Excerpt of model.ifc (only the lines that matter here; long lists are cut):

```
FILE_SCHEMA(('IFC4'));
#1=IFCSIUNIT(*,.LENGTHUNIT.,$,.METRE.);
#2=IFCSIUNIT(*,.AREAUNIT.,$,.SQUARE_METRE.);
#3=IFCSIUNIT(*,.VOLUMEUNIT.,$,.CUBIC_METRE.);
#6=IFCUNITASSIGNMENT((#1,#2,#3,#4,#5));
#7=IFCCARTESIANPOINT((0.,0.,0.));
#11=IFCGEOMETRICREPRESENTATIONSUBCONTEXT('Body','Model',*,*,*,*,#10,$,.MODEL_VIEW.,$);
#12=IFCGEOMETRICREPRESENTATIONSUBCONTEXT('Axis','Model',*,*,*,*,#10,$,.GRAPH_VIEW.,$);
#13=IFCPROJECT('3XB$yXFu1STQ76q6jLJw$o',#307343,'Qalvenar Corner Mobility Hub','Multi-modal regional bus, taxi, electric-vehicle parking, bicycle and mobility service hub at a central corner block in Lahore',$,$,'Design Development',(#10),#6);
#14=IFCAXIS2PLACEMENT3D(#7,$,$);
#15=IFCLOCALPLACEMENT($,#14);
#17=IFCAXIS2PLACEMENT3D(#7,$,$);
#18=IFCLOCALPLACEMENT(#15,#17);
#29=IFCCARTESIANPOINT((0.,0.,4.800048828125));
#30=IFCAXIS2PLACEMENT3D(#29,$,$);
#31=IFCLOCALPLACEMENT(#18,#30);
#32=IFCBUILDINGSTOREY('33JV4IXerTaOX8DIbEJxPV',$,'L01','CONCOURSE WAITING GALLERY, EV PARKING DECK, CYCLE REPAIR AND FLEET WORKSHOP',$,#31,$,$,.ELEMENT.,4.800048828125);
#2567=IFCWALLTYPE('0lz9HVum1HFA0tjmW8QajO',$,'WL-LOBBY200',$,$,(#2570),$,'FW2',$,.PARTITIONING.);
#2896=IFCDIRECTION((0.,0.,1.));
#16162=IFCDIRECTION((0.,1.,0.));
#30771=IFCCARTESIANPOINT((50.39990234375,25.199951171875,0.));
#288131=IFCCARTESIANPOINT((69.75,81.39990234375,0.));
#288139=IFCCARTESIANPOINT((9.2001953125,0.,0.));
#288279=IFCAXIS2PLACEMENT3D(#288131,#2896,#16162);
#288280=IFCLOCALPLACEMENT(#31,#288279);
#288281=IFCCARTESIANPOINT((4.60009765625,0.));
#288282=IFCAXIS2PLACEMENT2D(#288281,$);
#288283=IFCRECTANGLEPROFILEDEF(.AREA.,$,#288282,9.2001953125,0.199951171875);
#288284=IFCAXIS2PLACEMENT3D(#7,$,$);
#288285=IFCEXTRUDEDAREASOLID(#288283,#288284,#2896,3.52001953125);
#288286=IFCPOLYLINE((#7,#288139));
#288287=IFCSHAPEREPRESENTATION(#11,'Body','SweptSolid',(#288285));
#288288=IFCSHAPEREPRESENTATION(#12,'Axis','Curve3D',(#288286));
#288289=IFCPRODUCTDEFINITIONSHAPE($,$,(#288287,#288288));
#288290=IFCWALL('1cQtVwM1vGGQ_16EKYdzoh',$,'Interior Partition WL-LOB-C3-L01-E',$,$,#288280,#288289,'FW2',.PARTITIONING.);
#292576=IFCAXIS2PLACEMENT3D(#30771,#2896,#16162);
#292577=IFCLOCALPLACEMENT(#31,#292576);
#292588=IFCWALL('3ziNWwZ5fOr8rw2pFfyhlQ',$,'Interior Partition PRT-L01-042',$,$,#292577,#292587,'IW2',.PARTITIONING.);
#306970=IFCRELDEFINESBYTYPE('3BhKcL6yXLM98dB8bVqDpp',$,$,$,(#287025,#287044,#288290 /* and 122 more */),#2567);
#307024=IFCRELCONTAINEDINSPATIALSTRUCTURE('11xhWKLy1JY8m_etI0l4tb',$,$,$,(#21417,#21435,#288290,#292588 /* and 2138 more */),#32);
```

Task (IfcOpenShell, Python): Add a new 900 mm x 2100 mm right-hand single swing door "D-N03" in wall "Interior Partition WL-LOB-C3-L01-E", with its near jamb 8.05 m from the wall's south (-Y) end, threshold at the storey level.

```python
import numpy as np
import ifcopenshell
import ifcopenshell.api.feature
import ifcopenshell.api.geometry
import ifcopenshell.api.root
import ifcopenshell.api.spatial
import ifcopenshell.geom
import ifcopenshell.util.element
import ifcopenshell.util.placement
import ifcopenshell.util.representation
import ifcopenshell.util.shape
import ifcopenshell.util.unit

model = ifcopenshell.open("model.ifc")
unit_scale = ifcopenshell.util.unit.calculate_unit_scale(model)
settings = ifcopenshell.geom.settings()


def volume(element):
    """Net volume in cubic metres, openings subtracted."""
    shape = ifcopenshell.geom.create_shape(settings, element)
    return ifcopenshell.util.shape.get_volume(shape.geometry)


wall = model.by_guid("1cQtVwM1vGGQ_16EKYdzoh")
storey = ifcopenshell.util.element.get_container(wall, ifc_class="IfcBuildingStorey")
context = ifcopenshell.util.representation.get_context(model, "Model", "Body", "MODEL_VIEW")
before = volume(wall)

width, height, from_end, sill = 0.9, 2.1, 8.05, 0.0  # metres

# The wall runs along its own X axis, and the end named is its -X end.
wall_shape = ifcopenshell.geom.create_shape(settings, wall)
x, y, z = ifcopenshell.util.shape.get_vertices(wall_shape.geometry).T
start = x.min() + from_end
face, thickness = float(y.min()), float(y.max() - y.min())
wall_matrix = ifcopenshell.util.placement.get_local_placement(wall.ObjectPlacement)
level = ifcopenshell.util.placement.get_local_placement(storey.ObjectPlacement)[2, 3]


def in_wall(x, y):
    """Placement at x, y metres in the wall's axes, at sill height."""
    matrix = wall_matrix.copy()
    matrix[:, 3] = wall_matrix @ np.array([x / unit_scale, y / unit_scale, 0.0, 1.0])
    matrix[2, 3] = level + sill / unit_scale
    return matrix


# Opening: a box that overshoots both wall faces by 50 mm.
opening = ifcopenshell.api.root.create_entity(model, ifc_class="IfcOpeningElement", predefined_type="OPENING")
box = ifcopenshell.api.geometry.add_wall_representation(
    model, context=context, length=width, height=height, thickness=thickness + 0.1
)
ifcopenshell.api.geometry.assign_representation(model, product=opening, representation=box)
ifcopenshell.api.geometry.edit_object_placement(model, product=opening, matrix=in_wall(start, face - 0.05), is_si=False)
ifcopenshell.api.feature.add_feature(model, feature=opening, element=wall)

door = ifcopenshell.api.root.create_entity(model, ifc_class="IfcDoor", name="D-N03", predefined_type="DOOR")
door.OverallWidth, door.OverallHeight = width / unit_scale, height / unit_scale
door.OperationType = "SINGLE_SWING_RIGHT"
body = ifcopenshell.api.geometry.add_door_representation(
    model,
    context=context,
    overall_width=door.OverallWidth,
    overall_height=door.OverallHeight,
    operation_type="SINGLE_SWING_RIGHT",
    lining_properties={"LiningDepth": thickness / unit_scale, "ThresholdDepth": thickness / unit_scale},
)
ifcopenshell.api.geometry.assign_representation(model, product=door, representation=body)
ifcopenshell.api.spatial.assign_container(model, products=[door], relating_structure=storey)
ifcopenshell.api.feature.add_filling(model, opening=opening, element=door)

# The lining spans the wall, so the door starts at the wall face.
ifcopenshell.api.geometry.edit_object_placement(model, product=door, matrix=in_wall(start, face), is_si=False)

after = volume(wall)

print(f"wall volume {before:.3f} -> {after:.3f} m3")

model.write("model_edited.ifc")
```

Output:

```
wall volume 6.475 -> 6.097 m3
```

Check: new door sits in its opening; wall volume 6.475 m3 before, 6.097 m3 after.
